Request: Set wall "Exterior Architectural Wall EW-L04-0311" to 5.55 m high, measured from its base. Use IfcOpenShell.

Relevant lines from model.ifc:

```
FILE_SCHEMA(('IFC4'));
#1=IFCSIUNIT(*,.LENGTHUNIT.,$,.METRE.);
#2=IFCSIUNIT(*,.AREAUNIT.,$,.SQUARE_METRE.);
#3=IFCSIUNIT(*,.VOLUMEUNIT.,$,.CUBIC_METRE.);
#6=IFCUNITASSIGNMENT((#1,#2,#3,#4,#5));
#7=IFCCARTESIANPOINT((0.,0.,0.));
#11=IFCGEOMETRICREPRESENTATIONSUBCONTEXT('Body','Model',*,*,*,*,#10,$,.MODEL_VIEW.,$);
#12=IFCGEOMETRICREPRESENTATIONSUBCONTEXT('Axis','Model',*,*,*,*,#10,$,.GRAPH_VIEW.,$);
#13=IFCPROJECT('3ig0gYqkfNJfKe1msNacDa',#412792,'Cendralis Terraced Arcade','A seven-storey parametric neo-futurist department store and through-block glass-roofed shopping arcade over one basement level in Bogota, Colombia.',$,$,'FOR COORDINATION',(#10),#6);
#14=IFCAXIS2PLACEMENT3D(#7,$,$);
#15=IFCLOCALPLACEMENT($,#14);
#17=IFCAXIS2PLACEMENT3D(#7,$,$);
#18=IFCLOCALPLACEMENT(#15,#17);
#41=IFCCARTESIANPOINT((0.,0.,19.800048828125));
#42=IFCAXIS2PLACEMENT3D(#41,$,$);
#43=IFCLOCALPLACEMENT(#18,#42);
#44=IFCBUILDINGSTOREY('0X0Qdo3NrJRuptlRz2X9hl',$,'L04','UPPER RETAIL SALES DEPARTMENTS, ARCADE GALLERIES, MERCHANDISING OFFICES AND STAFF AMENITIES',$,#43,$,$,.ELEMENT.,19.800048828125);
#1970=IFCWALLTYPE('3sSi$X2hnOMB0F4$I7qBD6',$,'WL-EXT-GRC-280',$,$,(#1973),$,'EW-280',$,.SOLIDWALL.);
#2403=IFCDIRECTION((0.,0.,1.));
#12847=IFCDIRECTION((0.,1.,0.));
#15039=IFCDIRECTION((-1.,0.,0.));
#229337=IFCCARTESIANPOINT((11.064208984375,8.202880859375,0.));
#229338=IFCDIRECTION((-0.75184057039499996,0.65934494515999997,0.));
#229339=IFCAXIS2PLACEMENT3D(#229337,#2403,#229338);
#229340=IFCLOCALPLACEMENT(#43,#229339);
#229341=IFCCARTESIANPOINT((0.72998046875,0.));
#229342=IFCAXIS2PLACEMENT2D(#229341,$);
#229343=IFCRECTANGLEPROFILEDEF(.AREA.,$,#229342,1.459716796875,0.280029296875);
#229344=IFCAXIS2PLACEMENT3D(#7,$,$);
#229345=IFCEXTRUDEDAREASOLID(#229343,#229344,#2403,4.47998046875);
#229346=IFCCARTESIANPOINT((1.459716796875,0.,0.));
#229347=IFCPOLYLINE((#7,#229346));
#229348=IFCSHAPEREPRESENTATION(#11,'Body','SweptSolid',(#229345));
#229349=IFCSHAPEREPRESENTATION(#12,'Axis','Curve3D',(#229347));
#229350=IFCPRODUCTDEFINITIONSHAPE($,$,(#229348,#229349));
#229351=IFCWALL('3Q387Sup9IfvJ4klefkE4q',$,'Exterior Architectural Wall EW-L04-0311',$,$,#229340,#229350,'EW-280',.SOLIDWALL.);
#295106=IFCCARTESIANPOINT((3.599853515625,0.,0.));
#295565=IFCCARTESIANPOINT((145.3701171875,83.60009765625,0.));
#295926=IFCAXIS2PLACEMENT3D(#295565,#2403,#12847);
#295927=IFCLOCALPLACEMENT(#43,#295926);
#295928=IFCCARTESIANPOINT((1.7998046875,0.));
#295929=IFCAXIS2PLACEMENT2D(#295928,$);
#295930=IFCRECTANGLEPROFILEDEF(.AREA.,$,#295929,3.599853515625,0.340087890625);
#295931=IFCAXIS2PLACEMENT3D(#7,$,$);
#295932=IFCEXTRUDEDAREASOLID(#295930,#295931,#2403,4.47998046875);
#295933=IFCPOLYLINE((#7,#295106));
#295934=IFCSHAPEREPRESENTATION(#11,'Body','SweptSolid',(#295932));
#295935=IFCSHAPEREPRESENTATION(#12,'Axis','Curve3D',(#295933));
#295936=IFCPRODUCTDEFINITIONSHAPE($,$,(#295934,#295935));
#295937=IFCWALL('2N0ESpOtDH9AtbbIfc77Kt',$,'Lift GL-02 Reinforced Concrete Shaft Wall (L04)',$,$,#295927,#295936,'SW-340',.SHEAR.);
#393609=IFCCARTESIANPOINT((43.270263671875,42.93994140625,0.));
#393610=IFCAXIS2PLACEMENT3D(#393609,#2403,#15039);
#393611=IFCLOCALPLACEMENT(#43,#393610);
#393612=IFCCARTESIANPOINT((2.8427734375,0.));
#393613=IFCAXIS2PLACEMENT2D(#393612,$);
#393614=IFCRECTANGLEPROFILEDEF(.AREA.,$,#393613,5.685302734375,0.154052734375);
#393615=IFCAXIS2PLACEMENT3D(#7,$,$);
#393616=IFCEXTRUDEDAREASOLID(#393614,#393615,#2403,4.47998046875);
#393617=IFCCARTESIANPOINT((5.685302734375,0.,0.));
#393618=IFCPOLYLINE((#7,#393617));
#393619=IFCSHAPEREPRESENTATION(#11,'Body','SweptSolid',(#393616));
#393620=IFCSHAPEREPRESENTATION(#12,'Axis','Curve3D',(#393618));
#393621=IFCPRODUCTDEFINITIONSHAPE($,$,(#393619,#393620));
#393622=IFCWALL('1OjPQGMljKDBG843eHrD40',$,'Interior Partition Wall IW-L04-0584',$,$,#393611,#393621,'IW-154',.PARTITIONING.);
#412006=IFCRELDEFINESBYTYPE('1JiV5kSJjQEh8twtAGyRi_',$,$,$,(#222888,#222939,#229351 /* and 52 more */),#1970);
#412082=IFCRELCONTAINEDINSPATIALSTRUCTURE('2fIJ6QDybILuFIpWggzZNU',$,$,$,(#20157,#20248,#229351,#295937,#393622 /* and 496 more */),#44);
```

```python
import ifcopenshell
import ifcopenshell.geom
import ifcopenshell.util.representation
import ifcopenshell.util.shape

model = ifcopenshell.open("model.ifc")
settings = ifcopenshell.geom.settings()


def volume(element):
    """Net volume in cubic metres, openings subtracted."""
    shape = ifcopenshell.geom.create_shape(settings, element)
    return ifcopenshell.util.shape.get_volume(shape.geometry)


wall = model.by_guid("3Q387Sup9IfvJ4klefkE4q")
before = volume(wall)

body = ifcopenshell.util.representation.get_representation(wall, "Model", "Body")
solid = body.Items[0]
old_height = solid.Depth
solid.Depth = 5.55
after = volume(wall)

print(f"height {old_height:g} -> {solid.Depth:g}, volume {before:.3f} -> {after:.3f} m3")

model.write("model_edited.ifc")
```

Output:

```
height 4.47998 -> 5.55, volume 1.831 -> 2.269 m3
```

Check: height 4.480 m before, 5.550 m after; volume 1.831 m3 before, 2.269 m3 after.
